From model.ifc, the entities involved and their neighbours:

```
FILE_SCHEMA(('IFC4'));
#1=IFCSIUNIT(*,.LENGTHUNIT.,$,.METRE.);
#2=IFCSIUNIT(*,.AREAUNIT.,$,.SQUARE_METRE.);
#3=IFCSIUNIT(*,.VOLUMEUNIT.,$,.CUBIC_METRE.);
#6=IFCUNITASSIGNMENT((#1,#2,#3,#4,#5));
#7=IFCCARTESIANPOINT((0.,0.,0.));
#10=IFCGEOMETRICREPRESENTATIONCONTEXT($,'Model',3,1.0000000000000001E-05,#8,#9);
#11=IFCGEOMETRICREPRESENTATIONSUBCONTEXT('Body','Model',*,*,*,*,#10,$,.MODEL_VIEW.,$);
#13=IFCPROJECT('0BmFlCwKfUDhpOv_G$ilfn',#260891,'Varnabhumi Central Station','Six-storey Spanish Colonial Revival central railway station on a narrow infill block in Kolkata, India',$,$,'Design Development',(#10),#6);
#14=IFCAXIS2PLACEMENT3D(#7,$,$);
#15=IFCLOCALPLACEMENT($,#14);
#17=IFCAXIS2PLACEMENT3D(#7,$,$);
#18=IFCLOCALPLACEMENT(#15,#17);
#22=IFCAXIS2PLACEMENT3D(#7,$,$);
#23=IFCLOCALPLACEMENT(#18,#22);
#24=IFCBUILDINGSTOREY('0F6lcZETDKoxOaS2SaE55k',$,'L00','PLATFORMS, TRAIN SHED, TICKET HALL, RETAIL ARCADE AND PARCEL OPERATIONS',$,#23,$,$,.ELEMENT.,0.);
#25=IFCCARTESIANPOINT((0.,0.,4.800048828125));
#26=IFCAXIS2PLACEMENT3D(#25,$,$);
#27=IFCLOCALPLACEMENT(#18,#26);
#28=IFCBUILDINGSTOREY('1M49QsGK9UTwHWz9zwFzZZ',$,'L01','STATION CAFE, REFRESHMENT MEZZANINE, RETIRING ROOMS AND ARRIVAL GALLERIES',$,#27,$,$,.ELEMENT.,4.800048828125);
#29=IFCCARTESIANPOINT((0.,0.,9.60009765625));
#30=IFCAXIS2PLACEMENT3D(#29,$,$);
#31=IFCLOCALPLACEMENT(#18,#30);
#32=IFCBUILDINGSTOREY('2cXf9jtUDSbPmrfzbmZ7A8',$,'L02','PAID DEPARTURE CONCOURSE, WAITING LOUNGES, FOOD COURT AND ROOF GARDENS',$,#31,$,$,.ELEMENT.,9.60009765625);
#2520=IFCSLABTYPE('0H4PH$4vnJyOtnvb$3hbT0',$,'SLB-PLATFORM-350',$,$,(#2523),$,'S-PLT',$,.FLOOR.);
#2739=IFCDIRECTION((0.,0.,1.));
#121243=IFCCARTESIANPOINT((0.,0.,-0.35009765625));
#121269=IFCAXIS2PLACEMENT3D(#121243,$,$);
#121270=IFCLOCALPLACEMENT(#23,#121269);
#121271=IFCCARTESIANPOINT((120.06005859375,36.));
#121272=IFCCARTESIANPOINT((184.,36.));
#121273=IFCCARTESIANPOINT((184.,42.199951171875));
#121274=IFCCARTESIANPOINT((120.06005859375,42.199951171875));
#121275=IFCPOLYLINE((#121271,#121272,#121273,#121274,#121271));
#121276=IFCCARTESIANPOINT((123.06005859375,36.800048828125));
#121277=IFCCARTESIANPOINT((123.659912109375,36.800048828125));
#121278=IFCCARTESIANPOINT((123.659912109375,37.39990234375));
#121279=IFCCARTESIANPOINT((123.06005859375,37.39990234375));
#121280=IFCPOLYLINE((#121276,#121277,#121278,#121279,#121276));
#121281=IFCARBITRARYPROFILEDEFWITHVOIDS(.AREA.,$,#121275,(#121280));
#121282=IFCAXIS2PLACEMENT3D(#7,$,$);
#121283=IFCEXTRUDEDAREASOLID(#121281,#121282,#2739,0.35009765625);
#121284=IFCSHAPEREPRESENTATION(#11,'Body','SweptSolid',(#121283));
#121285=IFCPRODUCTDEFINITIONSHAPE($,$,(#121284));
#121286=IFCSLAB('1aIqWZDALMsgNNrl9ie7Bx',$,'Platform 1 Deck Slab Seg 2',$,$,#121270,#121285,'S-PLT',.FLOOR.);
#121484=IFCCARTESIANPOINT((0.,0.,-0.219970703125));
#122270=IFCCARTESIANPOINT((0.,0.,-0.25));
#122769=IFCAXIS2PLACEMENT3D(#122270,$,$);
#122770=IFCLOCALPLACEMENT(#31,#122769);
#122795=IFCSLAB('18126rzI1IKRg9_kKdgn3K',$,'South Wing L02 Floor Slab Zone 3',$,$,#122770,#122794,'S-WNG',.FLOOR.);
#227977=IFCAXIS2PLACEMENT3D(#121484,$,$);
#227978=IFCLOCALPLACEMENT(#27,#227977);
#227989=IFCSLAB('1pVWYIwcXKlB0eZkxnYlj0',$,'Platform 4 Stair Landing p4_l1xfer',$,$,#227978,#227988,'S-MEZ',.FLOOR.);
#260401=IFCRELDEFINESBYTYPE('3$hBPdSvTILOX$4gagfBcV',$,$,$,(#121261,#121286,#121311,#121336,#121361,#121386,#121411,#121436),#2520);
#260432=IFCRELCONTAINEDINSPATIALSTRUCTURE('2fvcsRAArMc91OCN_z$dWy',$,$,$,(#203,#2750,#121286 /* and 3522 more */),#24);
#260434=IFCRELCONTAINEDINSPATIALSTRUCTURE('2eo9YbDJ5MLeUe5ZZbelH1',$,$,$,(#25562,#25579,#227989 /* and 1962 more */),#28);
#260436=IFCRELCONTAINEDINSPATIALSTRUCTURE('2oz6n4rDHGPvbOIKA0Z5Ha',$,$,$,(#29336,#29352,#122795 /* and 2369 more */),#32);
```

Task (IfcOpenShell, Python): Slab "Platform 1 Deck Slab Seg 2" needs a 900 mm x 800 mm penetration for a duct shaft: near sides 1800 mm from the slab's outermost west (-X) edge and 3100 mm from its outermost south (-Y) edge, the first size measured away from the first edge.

```python
import numpy as np
import ifcopenshell
import ifcopenshell.api.feature
import ifcopenshell.api.geometry
import ifcopenshell.api.root
import ifcopenshell.geom
import ifcopenshell.util.placement
import ifcopenshell.util.representation
import ifcopenshell.util.shape
import ifcopenshell.util.unit

model = ifcopenshell.open("model.ifc")
unit_scale = ifcopenshell.util.unit.calculate_unit_scale(model)
settings = ifcopenshell.geom.settings()


def volume(element):
    """Net volume in cubic metres, openings subtracted."""
    shape = ifcopenshell.geom.create_shape(settings, element)
    return ifcopenshell.util.shape.get_volume(shape.geometry)


slab = model.by_id(121286)
before = volume(slab)

# Extent in the slab's own axes, in metres. The edges named are its -X and -Y sides.
slab_shape = ifcopenshell.geom.create_shape(settings, slab)
vertices = ifcopenshell.util.shape.get_vertices(slab_shape.geometry)
x_min, y_min, bottom = vertices.min(axis=0)
top = vertices[:, 2].max()

opening = ifcopenshell.api.root.create_entity(model, ifc_class="IfcOpeningElement", name="Duct shaft opening", predefined_type="OPENING")
context = ifcopenshell.util.representation.get_context(model, "Model", "Body", "MODEL_VIEW")
width, depth = 0.9, 0.8
outline = [(0.0, 0.0), (width, 0.0), (width, depth), (0.0, depth), (0.0, 0.0)]
# Overshoot both faces by 50 mm so the cut is clean.
shape = ifcopenshell.api.geometry.add_slab_representation(
    model, context=context, depth=top - bottom + 0.1, polyline=outline
)
ifcopenshell.api.geometry.assign_representation(model, product=opening, representation=shape)

matrix = ifcopenshell.util.placement.get_local_placement(slab.ObjectPlacement)
matrix[:, 3] = matrix @ np.append(np.array([x_min + 1.8, y_min + 3.1, bottom - 0.05]) / unit_scale, 1.0)
ifcopenshell.api.geometry.edit_object_placement(model, product=opening, matrix=matrix, is_si=False)
ifcopenshell.api.feature.add_feature(model, feature=opening, element=slab)

after = volume(slab)

print(f"slab volume {before:.3f} -> {after:.3f} m3")

model.write("model_rev.ifc")
```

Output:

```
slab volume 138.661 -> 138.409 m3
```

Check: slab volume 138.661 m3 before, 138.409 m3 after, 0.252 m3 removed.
